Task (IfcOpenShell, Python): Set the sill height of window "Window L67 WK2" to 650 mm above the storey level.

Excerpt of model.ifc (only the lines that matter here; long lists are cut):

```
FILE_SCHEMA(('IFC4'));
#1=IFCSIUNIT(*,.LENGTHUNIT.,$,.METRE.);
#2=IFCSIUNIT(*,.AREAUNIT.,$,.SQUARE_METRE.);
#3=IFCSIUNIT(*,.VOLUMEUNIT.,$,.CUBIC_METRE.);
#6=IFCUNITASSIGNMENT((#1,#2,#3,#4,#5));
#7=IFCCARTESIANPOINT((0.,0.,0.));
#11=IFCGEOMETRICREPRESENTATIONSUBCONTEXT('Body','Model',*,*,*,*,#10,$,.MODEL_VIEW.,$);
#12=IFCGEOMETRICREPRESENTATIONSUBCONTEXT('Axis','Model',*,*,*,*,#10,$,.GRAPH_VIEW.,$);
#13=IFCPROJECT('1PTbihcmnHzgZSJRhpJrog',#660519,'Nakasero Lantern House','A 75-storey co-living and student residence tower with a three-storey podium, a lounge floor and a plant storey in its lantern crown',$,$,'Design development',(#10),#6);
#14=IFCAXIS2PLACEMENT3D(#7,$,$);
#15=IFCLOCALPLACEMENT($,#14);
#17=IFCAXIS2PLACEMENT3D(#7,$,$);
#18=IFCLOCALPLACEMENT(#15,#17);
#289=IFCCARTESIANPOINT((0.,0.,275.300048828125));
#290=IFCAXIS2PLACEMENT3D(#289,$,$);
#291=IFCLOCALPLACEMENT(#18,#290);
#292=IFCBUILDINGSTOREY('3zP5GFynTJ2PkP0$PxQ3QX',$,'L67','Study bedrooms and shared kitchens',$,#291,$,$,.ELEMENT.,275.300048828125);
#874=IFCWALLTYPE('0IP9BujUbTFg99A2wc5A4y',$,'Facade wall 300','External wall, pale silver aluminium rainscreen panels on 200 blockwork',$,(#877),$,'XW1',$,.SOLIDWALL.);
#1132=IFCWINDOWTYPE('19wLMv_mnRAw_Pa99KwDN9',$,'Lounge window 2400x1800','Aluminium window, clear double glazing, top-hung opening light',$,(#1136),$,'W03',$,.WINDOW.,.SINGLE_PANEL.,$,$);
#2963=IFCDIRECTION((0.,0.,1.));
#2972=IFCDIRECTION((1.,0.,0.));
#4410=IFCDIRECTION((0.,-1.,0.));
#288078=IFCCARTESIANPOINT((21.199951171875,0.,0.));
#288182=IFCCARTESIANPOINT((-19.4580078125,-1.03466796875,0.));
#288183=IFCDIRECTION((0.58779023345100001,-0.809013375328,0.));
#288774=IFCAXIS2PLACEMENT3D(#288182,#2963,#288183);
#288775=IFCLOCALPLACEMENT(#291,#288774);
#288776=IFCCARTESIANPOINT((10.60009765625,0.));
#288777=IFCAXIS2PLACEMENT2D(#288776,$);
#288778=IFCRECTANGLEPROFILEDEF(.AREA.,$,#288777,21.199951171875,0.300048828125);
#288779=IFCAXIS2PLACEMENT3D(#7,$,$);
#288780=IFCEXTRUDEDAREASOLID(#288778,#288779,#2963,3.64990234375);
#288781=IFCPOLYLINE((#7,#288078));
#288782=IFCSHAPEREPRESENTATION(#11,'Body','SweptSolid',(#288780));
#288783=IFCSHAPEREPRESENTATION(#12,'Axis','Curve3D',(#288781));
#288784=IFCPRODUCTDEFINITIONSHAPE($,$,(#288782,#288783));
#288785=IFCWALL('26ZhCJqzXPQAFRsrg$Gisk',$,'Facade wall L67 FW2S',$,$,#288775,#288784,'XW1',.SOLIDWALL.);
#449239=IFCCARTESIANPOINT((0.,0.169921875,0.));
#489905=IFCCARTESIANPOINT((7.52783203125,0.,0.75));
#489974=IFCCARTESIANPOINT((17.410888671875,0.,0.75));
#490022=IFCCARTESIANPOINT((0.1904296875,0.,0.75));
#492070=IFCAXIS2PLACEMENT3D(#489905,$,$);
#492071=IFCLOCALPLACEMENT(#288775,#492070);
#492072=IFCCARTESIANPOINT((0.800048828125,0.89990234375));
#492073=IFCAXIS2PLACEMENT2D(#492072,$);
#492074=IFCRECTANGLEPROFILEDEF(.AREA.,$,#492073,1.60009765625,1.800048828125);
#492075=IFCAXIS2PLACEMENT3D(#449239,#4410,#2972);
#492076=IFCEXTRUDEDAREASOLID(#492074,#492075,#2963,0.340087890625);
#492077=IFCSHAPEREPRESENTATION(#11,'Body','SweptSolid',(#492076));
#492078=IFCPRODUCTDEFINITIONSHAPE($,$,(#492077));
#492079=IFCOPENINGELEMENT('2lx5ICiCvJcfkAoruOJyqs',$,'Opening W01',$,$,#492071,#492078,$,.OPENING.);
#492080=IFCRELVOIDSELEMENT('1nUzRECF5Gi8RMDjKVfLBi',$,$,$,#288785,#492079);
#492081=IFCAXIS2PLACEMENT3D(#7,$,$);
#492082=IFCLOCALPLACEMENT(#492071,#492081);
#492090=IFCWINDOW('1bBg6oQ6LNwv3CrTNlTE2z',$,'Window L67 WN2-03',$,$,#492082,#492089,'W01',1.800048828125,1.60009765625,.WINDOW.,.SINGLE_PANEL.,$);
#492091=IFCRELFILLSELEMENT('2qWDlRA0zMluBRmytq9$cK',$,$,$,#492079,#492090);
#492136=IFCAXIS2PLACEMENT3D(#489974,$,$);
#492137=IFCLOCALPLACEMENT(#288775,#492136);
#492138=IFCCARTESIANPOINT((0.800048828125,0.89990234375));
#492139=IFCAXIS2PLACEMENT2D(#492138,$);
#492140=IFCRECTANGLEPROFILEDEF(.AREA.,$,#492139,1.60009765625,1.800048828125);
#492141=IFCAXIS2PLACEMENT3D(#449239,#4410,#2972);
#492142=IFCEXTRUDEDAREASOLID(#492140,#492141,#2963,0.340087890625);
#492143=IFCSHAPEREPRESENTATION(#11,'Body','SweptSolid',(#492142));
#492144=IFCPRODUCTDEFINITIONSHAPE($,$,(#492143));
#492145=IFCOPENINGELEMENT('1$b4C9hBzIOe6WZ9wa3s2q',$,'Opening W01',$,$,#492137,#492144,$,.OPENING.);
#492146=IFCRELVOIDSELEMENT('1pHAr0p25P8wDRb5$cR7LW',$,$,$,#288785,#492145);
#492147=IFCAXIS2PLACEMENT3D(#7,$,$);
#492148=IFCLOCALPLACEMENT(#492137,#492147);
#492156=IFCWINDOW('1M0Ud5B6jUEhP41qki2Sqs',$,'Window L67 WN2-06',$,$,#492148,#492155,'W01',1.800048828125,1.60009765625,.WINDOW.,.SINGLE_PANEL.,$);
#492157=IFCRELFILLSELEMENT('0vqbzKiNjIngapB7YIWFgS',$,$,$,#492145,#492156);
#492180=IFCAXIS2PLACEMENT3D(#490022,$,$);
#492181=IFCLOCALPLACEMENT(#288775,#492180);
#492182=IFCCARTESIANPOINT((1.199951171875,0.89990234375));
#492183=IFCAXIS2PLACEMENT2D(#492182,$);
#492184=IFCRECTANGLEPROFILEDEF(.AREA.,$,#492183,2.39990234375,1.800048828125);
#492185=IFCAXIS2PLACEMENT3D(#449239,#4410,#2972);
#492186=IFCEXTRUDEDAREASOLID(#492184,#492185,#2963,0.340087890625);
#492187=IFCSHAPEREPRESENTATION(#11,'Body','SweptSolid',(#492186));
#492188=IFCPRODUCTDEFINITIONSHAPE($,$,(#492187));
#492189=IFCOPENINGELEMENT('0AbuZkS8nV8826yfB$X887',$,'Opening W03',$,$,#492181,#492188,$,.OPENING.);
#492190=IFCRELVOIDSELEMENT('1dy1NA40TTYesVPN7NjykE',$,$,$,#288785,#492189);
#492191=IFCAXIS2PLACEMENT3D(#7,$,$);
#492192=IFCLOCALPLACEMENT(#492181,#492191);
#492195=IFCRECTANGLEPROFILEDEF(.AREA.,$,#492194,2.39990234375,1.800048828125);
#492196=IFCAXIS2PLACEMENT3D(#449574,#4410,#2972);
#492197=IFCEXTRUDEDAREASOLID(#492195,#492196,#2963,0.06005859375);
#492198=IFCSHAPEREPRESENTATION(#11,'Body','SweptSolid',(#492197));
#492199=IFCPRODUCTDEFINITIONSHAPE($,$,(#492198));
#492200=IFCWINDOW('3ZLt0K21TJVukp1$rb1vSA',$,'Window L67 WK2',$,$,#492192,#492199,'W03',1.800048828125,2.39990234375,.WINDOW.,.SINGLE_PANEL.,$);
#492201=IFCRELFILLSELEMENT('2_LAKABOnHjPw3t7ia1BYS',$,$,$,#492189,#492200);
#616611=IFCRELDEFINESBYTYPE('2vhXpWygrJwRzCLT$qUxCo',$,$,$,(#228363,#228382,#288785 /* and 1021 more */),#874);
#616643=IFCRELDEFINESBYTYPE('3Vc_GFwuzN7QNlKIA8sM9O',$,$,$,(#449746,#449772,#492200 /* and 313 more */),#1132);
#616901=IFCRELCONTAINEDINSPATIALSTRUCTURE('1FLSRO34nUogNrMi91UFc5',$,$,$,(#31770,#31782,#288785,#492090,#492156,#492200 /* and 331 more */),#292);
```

```python
import numpy as np
import ifcopenshell
import ifcopenshell.api.geometry
import ifcopenshell.geom
import ifcopenshell.util.element
import ifcopenshell.util.placement
import ifcopenshell.util.shape
import ifcopenshell.util.unit

model = ifcopenshell.open("model.ifc")
unit_scale = ifcopenshell.util.unit.calculate_unit_scale(model)

window = model.by_guid("3ZLt0K21TJVukp1$rb1vSA")
opening = window.FillsVoids[0].RelatingOpeningElement
storey = ifcopenshell.util.element.get_container(window, ifc_class="IfcBuildingStorey")
level = ifcopenshell.util.placement.get_local_placement(storey.ObjectPlacement)[2, 3]

# The opening's origin need not be at the sill, so measure its lowest point.
shape = ifcopenshell.geom.create_shape(ifcopenshell.geom.settings(), opening)
bottom = ifcopenshell.util.shape.get_shape_bottom_elevation(shape, shape.geometry) / unit_scale
dz = level + 0.65 - bottom

shift = np.array([0.0, 0.0, dz])
# The window is placed relative to its opening, so it follows when the opening moves.
matrix = ifcopenshell.util.placement.get_local_placement(opening.ObjectPlacement)
matrix[:3, 3] += shift
ifcopenshell.api.geometry.edit_object_placement(
    model, product=opening, matrix=matrix, is_si=False, should_transform_children=True
)

print(f"moved by {dz * unit_scale:+.3f} m")

model.write("model-out.ifc")
```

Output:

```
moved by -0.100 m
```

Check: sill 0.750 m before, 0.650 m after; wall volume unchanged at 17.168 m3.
